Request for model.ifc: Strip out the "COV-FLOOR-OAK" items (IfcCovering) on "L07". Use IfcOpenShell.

First a look at what the model holds.

```python
import ifcopenshell
import ifcopenshell.util.element

model = ifcopenshell.open("model.ifc")
print(model.schema)
storey = next(s for s in model.by_type("IfcBuildingStorey") if s.Name == "L07")
coverings = [e for e in ifcopenshell.util.element.get_decomposition(storey) if e.is_a("IfcCovering")]
seen = {}
for e in coverings:
    element_type = ifcopenshell.util.element.get_type(e)
    name = element_type.Name if element_type not in (None, e) else None
    seen[name] = seen.get(name, 0) + 1
for name, count in sorted(seen.items(), key=str):
    print(count, "x", name)
```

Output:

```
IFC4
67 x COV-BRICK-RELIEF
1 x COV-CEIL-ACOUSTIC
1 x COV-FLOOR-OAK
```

```python
import ifcopenshell
import ifcopenshell.api.root
import ifcopenshell.util.element

model = ifcopenshell.open("model.ifc")

storey = next(s for s in model.by_type("IfcBuildingStorey") if s.Name == "L07")
coverings = [e for e in ifcopenshell.util.element.get_decomposition(storey) if e.is_a("IfcCovering")]
targets = [e for e in coverings if (t := ifcopenshell.util.element.get_type(e)) not in (None, e) and t.Name == "COV-FLOOR-OAK"]

for e in targets:
    ifcopenshell.api.root.remove_product(model, product=e)
print(len(targets), "removed")

model.write("model_edited.ifc")
```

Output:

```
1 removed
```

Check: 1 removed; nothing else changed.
